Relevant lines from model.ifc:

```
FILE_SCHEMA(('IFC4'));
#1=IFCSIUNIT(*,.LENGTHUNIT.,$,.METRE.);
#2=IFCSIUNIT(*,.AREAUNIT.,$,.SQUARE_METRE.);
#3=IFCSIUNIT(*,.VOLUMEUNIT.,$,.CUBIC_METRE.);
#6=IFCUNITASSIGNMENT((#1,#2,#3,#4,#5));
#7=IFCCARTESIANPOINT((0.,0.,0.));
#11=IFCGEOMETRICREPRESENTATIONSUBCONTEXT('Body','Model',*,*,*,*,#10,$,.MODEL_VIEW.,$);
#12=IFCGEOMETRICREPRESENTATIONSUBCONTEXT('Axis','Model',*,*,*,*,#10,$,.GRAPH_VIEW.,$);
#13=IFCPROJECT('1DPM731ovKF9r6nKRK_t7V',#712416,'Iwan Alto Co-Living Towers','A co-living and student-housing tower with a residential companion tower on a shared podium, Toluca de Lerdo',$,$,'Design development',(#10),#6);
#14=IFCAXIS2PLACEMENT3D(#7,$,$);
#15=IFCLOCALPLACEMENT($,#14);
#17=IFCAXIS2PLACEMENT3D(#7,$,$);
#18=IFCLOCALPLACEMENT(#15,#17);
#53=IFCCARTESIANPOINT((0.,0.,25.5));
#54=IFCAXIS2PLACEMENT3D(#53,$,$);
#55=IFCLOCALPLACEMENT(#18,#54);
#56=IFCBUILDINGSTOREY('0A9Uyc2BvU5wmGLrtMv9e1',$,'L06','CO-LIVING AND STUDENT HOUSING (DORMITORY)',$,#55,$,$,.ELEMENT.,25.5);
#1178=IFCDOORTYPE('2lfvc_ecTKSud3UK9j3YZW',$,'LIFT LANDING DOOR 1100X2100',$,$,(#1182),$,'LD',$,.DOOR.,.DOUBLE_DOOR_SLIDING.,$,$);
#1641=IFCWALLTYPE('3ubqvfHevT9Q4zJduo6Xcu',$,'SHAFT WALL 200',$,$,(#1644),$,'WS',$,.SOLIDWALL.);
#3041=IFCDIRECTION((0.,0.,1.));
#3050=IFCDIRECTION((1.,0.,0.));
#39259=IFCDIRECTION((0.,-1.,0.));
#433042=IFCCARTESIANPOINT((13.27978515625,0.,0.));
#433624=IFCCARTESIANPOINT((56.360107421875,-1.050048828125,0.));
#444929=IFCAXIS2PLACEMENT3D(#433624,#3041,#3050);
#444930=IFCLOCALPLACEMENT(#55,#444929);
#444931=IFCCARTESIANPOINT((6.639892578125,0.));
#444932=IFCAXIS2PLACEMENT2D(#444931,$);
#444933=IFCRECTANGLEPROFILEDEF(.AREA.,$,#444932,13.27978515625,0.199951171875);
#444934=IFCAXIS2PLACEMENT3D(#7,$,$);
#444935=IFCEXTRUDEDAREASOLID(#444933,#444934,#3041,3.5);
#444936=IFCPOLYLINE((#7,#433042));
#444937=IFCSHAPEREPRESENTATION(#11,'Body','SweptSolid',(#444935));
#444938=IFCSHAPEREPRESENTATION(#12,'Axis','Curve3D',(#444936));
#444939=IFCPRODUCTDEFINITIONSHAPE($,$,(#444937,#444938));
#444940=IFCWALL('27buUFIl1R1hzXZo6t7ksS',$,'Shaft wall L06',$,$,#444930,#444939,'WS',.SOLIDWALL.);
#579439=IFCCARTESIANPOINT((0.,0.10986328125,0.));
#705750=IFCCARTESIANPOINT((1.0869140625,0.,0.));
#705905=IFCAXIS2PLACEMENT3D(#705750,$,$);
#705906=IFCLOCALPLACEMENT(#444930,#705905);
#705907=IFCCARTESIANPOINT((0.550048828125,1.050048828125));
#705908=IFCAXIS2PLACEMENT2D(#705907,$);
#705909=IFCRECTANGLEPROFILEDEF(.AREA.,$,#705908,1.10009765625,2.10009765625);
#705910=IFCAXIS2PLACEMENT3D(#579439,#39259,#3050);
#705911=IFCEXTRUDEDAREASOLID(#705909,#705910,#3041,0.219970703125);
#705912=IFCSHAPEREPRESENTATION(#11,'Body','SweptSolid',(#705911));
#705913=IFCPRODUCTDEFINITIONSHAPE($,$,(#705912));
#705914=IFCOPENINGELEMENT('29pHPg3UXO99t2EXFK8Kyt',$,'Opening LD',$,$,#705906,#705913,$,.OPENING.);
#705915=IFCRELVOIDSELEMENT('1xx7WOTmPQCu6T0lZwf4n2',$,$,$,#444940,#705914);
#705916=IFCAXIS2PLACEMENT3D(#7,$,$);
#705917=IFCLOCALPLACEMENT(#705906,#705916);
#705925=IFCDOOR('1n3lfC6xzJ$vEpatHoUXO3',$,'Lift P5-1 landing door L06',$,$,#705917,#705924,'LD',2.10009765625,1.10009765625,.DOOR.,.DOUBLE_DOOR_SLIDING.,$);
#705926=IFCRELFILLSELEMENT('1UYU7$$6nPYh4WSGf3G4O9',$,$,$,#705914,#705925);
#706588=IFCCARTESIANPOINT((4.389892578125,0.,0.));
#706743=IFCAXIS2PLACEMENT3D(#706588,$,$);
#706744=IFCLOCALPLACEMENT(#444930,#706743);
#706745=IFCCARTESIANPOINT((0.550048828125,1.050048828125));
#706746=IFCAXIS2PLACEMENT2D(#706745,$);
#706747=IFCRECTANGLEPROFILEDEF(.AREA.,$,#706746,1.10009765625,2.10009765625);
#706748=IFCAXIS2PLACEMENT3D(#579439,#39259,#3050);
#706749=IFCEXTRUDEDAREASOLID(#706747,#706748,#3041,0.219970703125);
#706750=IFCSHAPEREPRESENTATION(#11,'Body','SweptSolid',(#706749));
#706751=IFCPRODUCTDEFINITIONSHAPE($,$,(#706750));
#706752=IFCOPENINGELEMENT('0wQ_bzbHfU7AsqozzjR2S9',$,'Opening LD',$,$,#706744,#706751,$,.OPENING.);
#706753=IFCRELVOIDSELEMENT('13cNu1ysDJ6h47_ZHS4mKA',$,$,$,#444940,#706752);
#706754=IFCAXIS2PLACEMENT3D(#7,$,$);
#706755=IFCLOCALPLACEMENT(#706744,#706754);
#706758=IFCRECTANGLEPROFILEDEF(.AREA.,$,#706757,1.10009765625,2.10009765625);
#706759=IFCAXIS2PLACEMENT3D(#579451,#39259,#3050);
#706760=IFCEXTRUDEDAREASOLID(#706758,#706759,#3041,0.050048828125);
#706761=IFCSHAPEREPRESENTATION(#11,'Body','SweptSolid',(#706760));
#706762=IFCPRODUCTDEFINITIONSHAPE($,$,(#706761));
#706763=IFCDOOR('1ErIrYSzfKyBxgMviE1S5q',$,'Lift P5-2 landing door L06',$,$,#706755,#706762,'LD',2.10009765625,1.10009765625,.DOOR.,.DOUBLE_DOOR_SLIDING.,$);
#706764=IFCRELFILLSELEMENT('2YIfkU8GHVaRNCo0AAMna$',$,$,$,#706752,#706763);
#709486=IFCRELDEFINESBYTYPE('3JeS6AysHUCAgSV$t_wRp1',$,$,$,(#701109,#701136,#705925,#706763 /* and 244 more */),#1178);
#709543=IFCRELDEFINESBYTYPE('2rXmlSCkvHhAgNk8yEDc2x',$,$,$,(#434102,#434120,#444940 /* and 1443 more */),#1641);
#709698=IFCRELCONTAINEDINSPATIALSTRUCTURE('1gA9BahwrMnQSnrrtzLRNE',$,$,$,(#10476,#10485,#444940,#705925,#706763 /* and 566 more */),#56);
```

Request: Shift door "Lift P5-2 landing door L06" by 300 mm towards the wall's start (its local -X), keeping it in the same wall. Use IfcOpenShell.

```python
import ifcopenshell
import ifcopenshell.api.geometry
import ifcopenshell.util.placement

model = ifcopenshell.open("model.ifc")

door = model.by_guid("1ErIrYSzfKyBxgMviE1S5q")
opening = door.FillsVoids[0].RelatingOpeningElement
wall = opening.VoidsElements[0].RelatingBuildingElement

wall_matrix = ifcopenshell.util.placement.get_local_placement(wall.ObjectPlacement)
shift = wall_matrix[:3, 0] * -0.3
before = ifcopenshell.util.placement.get_local_placement(door.ObjectPlacement)[:3, 3].copy()

# The door is placed relative to its opening, so it follows when the opening moves.
matrix = ifcopenshell.util.placement.get_local_placement(opening.ObjectPlacement)
matrix[:3, 3] += shift
ifcopenshell.api.geometry.edit_object_placement(
    model, product=opening, matrix=matrix, is_si=False, should_transform_children=True
)

after = ifcopenshell.util.placement.get_local_placement(door.ObjectPlacement)[:3, 3]
print("door moved by", (after - before).round(3) + 0.0)

model.write("model_rev.ifc")
```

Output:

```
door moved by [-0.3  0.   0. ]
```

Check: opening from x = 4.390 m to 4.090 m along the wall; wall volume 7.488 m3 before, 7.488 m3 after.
